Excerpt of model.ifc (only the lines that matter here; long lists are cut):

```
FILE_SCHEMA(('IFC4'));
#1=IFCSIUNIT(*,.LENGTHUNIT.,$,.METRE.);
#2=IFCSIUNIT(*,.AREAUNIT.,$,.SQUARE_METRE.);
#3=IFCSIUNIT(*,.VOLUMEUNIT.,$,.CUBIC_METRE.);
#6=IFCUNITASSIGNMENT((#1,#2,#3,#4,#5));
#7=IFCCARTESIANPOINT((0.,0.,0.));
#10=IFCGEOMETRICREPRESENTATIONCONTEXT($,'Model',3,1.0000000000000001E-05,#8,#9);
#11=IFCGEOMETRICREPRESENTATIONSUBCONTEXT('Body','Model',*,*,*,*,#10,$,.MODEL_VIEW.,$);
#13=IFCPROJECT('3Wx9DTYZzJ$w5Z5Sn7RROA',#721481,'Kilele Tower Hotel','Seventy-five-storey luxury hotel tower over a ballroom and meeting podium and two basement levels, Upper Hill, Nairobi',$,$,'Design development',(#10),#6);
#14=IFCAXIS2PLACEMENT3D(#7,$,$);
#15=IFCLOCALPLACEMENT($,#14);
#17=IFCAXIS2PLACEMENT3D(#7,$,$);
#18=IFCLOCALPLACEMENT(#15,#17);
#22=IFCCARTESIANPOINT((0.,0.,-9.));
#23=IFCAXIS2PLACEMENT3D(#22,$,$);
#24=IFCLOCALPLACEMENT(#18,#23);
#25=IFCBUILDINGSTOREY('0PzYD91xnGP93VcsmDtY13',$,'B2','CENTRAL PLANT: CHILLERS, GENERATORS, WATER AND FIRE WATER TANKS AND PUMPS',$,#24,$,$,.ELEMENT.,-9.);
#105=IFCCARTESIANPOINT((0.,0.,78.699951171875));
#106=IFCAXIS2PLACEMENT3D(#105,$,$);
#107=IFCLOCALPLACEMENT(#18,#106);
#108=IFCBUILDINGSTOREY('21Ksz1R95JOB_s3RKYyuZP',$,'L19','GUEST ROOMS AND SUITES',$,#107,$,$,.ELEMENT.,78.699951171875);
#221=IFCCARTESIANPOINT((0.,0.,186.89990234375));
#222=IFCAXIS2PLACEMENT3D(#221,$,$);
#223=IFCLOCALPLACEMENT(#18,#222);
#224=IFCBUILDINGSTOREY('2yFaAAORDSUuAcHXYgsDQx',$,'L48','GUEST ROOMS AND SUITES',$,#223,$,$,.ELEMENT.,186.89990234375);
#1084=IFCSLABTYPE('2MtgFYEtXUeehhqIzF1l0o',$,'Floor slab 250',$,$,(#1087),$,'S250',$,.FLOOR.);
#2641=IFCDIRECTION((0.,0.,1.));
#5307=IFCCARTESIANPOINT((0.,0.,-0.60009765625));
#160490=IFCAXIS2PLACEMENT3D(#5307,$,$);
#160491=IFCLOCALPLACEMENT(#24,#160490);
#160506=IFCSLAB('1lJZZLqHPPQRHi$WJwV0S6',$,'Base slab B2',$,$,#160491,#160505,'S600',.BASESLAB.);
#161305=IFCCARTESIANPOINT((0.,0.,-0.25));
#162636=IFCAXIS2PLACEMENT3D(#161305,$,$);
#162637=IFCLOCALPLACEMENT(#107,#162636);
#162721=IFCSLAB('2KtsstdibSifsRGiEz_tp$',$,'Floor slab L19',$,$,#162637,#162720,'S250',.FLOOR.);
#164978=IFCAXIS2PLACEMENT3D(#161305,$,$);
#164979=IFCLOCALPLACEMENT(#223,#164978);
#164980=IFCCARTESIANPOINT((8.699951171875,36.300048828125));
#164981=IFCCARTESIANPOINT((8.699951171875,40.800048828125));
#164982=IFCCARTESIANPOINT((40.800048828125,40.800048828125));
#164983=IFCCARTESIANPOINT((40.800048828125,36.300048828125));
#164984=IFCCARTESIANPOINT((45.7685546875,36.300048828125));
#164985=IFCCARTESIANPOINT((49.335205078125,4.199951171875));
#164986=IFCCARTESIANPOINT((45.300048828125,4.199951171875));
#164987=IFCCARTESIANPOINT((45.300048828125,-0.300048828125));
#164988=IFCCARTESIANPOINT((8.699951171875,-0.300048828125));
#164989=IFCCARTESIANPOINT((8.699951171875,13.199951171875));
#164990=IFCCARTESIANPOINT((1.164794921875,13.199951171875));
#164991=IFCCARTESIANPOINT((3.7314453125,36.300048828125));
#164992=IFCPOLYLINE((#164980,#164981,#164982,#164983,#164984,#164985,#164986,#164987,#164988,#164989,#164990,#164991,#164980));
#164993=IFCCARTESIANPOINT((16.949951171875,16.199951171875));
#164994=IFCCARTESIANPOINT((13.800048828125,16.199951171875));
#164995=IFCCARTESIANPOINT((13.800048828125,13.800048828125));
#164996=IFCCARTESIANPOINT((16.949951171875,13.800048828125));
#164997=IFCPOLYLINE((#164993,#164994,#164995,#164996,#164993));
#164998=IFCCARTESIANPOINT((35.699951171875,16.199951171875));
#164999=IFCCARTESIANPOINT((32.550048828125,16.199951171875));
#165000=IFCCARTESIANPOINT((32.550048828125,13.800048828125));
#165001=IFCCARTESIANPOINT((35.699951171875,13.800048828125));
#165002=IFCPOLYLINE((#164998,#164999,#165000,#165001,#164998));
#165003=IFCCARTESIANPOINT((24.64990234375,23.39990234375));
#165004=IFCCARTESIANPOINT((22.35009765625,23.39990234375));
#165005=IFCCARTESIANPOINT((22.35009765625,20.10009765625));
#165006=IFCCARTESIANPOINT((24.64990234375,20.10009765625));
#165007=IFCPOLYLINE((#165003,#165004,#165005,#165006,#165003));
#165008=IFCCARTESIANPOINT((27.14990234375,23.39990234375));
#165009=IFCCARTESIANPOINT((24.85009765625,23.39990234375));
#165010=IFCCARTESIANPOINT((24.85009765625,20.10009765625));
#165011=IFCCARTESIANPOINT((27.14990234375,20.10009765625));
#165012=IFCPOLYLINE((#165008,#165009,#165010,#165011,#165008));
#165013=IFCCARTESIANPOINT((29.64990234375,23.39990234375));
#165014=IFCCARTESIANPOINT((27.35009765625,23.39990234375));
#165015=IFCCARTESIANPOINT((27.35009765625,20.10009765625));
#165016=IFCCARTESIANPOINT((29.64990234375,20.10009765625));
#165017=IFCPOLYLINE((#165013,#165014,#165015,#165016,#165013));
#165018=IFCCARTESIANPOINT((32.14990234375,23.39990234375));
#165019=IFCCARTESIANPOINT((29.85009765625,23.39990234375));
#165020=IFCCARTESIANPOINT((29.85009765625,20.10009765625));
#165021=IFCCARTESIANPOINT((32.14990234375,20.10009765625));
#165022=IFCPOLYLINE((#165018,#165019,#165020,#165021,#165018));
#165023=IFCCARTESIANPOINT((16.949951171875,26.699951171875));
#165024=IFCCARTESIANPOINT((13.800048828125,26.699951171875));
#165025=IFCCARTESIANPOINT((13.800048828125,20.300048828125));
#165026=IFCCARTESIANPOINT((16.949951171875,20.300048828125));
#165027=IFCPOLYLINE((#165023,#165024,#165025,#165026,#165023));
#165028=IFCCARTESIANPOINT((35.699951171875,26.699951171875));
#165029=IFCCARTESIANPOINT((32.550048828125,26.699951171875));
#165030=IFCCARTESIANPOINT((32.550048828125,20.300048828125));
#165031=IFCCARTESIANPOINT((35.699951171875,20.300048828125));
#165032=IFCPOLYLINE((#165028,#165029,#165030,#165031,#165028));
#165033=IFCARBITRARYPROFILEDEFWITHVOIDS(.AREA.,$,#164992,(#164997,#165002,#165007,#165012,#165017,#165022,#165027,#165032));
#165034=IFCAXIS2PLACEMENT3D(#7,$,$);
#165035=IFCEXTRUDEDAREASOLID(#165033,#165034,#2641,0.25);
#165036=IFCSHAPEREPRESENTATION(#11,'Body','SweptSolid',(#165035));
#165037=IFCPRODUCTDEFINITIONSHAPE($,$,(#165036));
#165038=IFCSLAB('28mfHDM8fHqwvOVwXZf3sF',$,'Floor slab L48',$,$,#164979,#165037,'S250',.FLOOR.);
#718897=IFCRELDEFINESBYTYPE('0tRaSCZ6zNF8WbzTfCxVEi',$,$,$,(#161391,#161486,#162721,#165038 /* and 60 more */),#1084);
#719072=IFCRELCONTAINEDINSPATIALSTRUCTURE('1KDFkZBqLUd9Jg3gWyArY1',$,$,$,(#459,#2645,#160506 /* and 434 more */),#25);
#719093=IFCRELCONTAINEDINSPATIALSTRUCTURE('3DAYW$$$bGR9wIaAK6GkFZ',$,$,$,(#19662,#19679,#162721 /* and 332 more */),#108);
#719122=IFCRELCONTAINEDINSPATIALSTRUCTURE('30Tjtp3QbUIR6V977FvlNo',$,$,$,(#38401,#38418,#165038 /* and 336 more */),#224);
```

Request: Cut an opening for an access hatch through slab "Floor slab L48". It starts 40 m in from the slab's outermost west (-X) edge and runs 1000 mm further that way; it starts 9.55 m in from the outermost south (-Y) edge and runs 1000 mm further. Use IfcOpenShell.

```python
import numpy as np
import ifcopenshell
import ifcopenshell.api.feature
import ifcopenshell.api.geometry
import ifcopenshell.api.root
import ifcopenshell.geom
import ifcopenshell.util.placement
import ifcopenshell.util.representation
import ifcopenshell.util.shape
import ifcopenshell.util.unit

model = ifcopenshell.open("model.ifc")
unit_scale = ifcopenshell.util.unit.calculate_unit_scale(model)
settings = ifcopenshell.geom.settings()


def volume(element):
    """Net volume in cubic metres, openings subtracted."""
    shape = ifcopenshell.geom.create_shape(settings, element)
    return ifcopenshell.util.shape.get_volume(shape.geometry)


slab = model.by_guid("28mfHDM8fHqwvOVwXZf3sF")
before = volume(slab)

# Extent in the slab's own axes, in metres. The edges named are its -X and -Y sides.
slab_shape = ifcopenshell.geom.create_shape(settings, slab)
vertices = ifcopenshell.util.shape.get_vertices(slab_shape.geometry)
x_min, y_min, bottom = vertices.min(axis=0)
top = vertices[:, 2].max()

opening = ifcopenshell.api.root.create_entity(model, ifc_class="IfcOpeningElement", name="Access hatch opening", predefined_type="OPENING")
context = ifcopenshell.util.representation.get_context(model, "Model", "Body", "MODEL_VIEW")
width, depth = 1, 1
outline = [(0.0, 0.0), (width, 0.0), (width, depth), (0.0, depth), (0.0, 0.0)]
# Overshoot both faces by 50 mm so the cut is clean.
shape = ifcopenshell.api.geometry.add_slab_representation(
    model, context=context, depth=top - bottom + 0.1, polyline=outline
)
ifcopenshell.api.geometry.assign_representation(model, product=opening, representation=shape)

matrix = ifcopenshell.util.placement.get_local_placement(slab.ObjectPlacement)
matrix[:, 3] = matrix @ np.append(np.array([x_min + 40, y_min + 9.55, bottom - 0.05]) / unit_scale, 1.0)
ifcopenshell.api.geometry.edit_object_placement(model, product=opening, matrix=matrix, is_si=False)
ifcopenshell.api.feature.add_feature(model, feature=opening, element=slab)

after = volume(slab)

print(f"slab volume {before:.3f} -> {after:.3f} m3")

model.write("model-out.ifc")
```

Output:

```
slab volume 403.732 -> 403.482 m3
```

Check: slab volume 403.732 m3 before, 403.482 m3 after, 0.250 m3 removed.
